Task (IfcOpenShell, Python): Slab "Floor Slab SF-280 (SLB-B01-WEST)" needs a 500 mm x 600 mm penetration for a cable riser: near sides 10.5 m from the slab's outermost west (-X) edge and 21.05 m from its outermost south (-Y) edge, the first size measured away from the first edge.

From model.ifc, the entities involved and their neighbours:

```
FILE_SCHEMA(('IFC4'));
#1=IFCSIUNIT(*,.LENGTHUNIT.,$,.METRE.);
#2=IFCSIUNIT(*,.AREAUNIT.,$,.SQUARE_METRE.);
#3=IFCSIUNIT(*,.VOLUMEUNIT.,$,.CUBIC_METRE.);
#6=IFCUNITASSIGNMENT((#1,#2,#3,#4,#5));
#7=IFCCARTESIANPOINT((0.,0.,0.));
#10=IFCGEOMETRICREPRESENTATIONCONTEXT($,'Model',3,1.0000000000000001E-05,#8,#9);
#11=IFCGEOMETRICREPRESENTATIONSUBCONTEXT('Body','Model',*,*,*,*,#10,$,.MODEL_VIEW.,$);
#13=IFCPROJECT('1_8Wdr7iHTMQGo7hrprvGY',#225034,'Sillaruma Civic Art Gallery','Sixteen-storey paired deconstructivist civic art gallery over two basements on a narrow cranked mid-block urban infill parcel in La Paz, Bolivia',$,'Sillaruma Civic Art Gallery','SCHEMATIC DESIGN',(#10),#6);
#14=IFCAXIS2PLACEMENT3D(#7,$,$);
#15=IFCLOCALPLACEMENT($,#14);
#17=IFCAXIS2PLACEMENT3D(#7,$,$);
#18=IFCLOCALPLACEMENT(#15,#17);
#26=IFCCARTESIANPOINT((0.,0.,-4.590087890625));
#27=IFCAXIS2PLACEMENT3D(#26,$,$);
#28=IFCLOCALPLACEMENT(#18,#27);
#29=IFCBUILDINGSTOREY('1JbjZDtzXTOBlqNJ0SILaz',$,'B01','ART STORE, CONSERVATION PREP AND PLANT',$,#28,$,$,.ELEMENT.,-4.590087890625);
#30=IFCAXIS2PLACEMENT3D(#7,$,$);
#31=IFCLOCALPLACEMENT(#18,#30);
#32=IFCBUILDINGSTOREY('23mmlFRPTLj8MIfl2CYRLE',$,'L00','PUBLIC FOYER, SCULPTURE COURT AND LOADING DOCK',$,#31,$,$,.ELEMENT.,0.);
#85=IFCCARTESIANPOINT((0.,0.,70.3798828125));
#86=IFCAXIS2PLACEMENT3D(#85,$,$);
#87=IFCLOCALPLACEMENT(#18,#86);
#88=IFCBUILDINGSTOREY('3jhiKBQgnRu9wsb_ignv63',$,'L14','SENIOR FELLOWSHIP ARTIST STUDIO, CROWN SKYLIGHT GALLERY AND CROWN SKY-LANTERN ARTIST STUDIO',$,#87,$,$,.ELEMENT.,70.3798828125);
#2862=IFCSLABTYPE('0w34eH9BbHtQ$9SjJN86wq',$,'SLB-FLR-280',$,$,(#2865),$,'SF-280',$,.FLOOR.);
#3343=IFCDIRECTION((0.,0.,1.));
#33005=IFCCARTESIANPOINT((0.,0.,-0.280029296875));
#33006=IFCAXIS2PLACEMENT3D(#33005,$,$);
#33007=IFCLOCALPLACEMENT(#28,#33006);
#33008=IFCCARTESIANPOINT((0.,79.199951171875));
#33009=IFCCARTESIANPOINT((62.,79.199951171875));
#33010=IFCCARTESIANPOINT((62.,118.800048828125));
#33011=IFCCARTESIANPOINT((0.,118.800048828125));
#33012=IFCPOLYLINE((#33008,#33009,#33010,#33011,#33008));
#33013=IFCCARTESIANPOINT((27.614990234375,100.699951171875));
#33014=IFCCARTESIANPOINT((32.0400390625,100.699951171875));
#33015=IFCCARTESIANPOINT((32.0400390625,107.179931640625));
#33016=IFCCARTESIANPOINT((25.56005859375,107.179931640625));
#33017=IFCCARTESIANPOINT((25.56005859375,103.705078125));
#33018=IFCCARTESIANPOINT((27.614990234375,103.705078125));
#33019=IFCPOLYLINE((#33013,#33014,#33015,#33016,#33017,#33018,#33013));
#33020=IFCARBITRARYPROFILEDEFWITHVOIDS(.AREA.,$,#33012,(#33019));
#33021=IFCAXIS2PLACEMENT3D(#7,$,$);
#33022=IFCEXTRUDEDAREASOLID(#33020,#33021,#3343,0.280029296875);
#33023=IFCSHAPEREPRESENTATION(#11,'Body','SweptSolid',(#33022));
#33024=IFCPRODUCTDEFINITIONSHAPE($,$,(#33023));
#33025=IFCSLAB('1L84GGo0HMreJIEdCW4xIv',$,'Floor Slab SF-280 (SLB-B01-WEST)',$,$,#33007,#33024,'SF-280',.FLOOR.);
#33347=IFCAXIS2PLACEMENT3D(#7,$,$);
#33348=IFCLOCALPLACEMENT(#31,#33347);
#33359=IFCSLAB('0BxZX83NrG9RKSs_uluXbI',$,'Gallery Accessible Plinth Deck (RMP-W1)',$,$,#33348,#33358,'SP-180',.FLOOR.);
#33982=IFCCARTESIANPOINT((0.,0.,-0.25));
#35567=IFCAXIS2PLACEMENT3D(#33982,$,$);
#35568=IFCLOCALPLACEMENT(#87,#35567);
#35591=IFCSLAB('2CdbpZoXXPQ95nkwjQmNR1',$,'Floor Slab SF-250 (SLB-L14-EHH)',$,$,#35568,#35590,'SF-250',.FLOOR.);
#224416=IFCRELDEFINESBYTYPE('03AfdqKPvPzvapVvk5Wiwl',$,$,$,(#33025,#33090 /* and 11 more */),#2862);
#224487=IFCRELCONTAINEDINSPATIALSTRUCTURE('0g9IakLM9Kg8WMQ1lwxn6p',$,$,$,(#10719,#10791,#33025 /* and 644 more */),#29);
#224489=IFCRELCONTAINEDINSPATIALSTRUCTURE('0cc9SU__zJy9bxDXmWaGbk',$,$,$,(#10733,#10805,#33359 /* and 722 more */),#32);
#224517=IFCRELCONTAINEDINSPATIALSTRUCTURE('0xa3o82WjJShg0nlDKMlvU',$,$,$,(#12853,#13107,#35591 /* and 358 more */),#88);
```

```python
import numpy as np
import ifcopenshell
import ifcopenshell.api.feature
import ifcopenshell.api.geometry
import ifcopenshell.api.root
import ifcopenshell.geom
import ifcopenshell.util.placement
import ifcopenshell.util.representation
import ifcopenshell.util.shape
import ifcopenshell.util.unit

model = ifcopenshell.open("model.ifc")
unit_scale = ifcopenshell.util.unit.calculate_unit_scale(model)
settings = ifcopenshell.geom.settings()


def volume(element):
    """Net volume in cubic metres, openings subtracted."""
    shape = ifcopenshell.geom.create_shape(settings, element)
    return ifcopenshell.util.shape.get_volume(shape.geometry)


slab = model.by_id(33025)
before = volume(slab)

# Extent in the slab's own axes, in metres. The edges named are its -X and -Y sides.
slab_shape = ifcopenshell.geom.create_shape(settings, slab)
vertices = ifcopenshell.util.shape.get_vertices(slab_shape.geometry)
x_min, y_min, bottom = vertices.min(axis=0)
top = vertices[:, 2].max()

opening = ifcopenshell.api.root.create_entity(model, ifc_class="IfcOpeningElement", name="Cable riser opening", predefined_type="OPENING")
context = ifcopenshell.util.representation.get_context(model, "Model", "Body", "MODEL_VIEW")
width, depth = 0.5, 0.6
outline = [(0.0, 0.0), (width, 0.0), (width, depth), (0.0, depth), (0.0, 0.0)]
# Overshoot both faces by 50 mm so the cut is clean.
shape = ifcopenshell.api.geometry.add_slab_representation(
    model, context=context, depth=top - bottom + 0.1, polyline=outline
)
ifcopenshell.api.geometry.assign_representation(model, product=opening, representation=shape)

matrix = ifcopenshell.util.placement.get_local_placement(slab.ObjectPlacement)
matrix[:, 3] = matrix @ np.append(np.array([x_min + 10.5, y_min + 21.05, bottom - 0.05]) / unit_scale, 1.0)
ifcopenshell.api.geometry.edit_object_placement(model, product=opening, matrix=matrix, is_si=False)
ifcopenshell.api.feature.add_feature(model, feature=opening, element=slab)

after = volume(slab)

print(f"slab volume {before:.3f} -> {after:.3f} m3")

model.write("model_updated.ifc")
```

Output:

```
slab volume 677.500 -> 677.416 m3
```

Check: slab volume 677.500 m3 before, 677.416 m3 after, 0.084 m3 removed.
